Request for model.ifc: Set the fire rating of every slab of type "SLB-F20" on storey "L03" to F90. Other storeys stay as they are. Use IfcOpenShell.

First a look at what the model holds.

```python
import ifcopenshell
import ifcopenshell.util.element

model = ifcopenshell.open("model.ifc")
print(model.schema)
storey = next(s for s in model.by_type("IfcBuildingStorey") if s.Name == "L03")
slabs = [e for e in ifcopenshell.util.element.get_decomposition(storey) if e.is_a("IfcSlab")]
seen = {}
for e in slabs:
    element_type = ifcopenshell.util.element.get_type(e)
    key = (element_type.Name if element_type != e and element_type else None, ifcopenshell.util.element.get_pset(e, "Pset_SlabCommon", "FireRating"))
    seen[key] = seen.get(key, 0) + 1
for (name, value), count in sorted(seen.items(), key=str):
    print(count, "x", name, "|", value)
```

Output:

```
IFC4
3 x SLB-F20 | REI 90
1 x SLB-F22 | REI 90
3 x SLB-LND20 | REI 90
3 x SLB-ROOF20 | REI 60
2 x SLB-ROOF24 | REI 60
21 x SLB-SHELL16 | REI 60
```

```python
import ifcopenshell
import ifcopenshell.api.pset
import ifcopenshell.util.element

model = ifcopenshell.open("model.ifc")

storey = next(s for s in model.by_type("IfcBuildingStorey") if s.Name == "L03")
slabs = [e for e in ifcopenshell.util.element.get_decomposition(storey) if e.is_a("IfcSlab")]

count = 0
for e in slabs:
    element_type = ifcopenshell.util.element.get_type(e)
    if element_type in (None, e) or element_type.Name != "SLB-F20":
        continue
    # add_pset returns the element's existing set when there is one.
    pset = ifcopenshell.api.pset.add_pset(model, product=e, name="Pset_SlabCommon")
    ifcopenshell.api.pset.edit_pset(model, pset=pset, properties={"FireRating": "F90"})
    count += 1

print(count, "slabs updated")

model.write("model_v2.ifc")
```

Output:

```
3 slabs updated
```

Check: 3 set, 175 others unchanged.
